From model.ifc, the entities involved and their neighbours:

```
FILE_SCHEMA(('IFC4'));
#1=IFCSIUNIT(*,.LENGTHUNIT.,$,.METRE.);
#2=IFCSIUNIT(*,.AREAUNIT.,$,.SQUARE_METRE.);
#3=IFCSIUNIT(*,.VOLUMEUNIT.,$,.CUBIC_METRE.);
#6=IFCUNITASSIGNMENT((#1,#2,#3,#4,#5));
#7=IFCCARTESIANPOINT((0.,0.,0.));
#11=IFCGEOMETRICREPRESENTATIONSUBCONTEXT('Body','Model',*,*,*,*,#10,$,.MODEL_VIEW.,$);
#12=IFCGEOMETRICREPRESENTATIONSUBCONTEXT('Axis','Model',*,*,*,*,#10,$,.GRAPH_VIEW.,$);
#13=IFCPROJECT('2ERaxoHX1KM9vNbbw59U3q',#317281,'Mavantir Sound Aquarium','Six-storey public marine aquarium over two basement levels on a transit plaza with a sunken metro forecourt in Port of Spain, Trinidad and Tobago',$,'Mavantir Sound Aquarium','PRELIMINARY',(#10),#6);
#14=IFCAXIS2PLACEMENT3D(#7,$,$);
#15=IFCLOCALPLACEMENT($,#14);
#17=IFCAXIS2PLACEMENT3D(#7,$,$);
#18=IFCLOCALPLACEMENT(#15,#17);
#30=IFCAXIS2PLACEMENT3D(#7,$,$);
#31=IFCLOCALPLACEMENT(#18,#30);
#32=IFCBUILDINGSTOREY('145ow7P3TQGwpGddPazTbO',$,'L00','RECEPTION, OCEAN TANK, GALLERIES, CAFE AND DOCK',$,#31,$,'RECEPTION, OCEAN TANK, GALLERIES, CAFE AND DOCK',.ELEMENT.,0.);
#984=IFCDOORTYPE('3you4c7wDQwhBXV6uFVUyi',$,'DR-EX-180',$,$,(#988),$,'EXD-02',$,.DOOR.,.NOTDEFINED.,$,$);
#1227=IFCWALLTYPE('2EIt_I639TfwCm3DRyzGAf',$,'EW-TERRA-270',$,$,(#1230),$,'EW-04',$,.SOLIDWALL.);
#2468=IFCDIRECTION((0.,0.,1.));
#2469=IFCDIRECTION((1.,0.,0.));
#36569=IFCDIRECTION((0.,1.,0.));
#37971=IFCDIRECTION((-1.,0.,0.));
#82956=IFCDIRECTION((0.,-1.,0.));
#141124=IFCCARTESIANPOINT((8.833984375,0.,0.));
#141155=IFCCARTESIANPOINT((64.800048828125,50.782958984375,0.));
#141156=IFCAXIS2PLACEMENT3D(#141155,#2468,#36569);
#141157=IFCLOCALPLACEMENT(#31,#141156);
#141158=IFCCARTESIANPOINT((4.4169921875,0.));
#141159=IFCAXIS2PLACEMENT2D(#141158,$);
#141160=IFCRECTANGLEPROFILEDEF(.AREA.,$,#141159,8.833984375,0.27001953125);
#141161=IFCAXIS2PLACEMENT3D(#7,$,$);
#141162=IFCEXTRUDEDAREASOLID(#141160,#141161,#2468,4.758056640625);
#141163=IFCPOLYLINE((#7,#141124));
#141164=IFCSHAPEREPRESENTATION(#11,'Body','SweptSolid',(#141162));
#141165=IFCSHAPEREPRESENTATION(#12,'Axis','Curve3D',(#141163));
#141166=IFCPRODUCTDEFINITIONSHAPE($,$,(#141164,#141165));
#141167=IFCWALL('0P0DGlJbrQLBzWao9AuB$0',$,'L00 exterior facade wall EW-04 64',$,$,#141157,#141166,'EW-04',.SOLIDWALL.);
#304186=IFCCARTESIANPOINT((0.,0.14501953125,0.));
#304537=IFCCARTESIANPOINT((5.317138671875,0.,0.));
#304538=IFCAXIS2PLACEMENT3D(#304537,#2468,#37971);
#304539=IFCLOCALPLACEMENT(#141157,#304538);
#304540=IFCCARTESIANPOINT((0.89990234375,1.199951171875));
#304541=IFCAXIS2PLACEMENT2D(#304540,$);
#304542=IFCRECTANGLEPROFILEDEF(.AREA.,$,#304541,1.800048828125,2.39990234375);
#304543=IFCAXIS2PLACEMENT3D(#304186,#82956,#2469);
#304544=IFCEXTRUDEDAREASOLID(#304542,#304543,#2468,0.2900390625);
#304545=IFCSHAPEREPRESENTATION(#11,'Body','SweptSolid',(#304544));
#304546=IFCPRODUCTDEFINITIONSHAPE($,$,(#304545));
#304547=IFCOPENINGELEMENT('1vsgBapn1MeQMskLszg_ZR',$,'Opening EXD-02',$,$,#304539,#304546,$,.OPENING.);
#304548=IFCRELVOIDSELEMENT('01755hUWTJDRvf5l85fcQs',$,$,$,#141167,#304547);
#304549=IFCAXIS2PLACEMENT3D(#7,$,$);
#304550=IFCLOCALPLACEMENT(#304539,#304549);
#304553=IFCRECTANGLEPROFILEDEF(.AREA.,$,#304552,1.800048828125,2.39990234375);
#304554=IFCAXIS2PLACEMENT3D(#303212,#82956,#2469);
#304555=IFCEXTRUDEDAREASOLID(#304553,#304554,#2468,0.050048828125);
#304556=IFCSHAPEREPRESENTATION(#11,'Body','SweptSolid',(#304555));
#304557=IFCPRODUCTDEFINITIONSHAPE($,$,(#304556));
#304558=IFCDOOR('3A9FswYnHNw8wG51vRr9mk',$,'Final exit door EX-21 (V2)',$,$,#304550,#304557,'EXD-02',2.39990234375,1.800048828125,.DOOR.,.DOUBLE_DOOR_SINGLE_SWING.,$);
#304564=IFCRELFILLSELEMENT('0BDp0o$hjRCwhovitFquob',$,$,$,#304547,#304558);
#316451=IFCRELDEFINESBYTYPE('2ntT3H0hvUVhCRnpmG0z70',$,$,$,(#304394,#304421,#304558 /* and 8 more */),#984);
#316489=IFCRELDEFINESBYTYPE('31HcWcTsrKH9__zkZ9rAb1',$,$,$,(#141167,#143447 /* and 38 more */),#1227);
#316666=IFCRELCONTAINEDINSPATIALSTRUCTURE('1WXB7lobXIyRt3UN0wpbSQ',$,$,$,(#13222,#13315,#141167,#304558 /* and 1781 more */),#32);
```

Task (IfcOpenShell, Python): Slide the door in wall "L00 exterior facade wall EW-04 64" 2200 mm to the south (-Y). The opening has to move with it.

```python
import ifcopenshell
import ifcopenshell.api.geometry
import ifcopenshell.util.placement

model = ifcopenshell.open("model.ifc")

door = model.by_guid("3A9FswYnHNw8wG51vRr9mk")
opening = door.FillsVoids[0].RelatingOpeningElement
wall = opening.VoidsElements[0].RelatingBuildingElement

wall_matrix = ifcopenshell.util.placement.get_local_placement(wall.ObjectPlacement)
shift = wall_matrix[:3, 0] * -2.2
before = ifcopenshell.util.placement.get_local_placement(door.ObjectPlacement)[:3, 3].copy()

# The door is placed relative to its opening, so it follows when the opening moves.
matrix = ifcopenshell.util.placement.get_local_placement(opening.ObjectPlacement)
matrix[:3, 3] += shift
ifcopenshell.api.geometry.edit_object_placement(
    model, product=opening, matrix=matrix, is_si=False, should_transform_children=True
)

after = ifcopenshell.util.placement.get_local_placement(door.ObjectPlacement)[:3, 3]
print("door moved by", (after - before).round(3) + 0.0)

model.write("model_v2.ifc")
```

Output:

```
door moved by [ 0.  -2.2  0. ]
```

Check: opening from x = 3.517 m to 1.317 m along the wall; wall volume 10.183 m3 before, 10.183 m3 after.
